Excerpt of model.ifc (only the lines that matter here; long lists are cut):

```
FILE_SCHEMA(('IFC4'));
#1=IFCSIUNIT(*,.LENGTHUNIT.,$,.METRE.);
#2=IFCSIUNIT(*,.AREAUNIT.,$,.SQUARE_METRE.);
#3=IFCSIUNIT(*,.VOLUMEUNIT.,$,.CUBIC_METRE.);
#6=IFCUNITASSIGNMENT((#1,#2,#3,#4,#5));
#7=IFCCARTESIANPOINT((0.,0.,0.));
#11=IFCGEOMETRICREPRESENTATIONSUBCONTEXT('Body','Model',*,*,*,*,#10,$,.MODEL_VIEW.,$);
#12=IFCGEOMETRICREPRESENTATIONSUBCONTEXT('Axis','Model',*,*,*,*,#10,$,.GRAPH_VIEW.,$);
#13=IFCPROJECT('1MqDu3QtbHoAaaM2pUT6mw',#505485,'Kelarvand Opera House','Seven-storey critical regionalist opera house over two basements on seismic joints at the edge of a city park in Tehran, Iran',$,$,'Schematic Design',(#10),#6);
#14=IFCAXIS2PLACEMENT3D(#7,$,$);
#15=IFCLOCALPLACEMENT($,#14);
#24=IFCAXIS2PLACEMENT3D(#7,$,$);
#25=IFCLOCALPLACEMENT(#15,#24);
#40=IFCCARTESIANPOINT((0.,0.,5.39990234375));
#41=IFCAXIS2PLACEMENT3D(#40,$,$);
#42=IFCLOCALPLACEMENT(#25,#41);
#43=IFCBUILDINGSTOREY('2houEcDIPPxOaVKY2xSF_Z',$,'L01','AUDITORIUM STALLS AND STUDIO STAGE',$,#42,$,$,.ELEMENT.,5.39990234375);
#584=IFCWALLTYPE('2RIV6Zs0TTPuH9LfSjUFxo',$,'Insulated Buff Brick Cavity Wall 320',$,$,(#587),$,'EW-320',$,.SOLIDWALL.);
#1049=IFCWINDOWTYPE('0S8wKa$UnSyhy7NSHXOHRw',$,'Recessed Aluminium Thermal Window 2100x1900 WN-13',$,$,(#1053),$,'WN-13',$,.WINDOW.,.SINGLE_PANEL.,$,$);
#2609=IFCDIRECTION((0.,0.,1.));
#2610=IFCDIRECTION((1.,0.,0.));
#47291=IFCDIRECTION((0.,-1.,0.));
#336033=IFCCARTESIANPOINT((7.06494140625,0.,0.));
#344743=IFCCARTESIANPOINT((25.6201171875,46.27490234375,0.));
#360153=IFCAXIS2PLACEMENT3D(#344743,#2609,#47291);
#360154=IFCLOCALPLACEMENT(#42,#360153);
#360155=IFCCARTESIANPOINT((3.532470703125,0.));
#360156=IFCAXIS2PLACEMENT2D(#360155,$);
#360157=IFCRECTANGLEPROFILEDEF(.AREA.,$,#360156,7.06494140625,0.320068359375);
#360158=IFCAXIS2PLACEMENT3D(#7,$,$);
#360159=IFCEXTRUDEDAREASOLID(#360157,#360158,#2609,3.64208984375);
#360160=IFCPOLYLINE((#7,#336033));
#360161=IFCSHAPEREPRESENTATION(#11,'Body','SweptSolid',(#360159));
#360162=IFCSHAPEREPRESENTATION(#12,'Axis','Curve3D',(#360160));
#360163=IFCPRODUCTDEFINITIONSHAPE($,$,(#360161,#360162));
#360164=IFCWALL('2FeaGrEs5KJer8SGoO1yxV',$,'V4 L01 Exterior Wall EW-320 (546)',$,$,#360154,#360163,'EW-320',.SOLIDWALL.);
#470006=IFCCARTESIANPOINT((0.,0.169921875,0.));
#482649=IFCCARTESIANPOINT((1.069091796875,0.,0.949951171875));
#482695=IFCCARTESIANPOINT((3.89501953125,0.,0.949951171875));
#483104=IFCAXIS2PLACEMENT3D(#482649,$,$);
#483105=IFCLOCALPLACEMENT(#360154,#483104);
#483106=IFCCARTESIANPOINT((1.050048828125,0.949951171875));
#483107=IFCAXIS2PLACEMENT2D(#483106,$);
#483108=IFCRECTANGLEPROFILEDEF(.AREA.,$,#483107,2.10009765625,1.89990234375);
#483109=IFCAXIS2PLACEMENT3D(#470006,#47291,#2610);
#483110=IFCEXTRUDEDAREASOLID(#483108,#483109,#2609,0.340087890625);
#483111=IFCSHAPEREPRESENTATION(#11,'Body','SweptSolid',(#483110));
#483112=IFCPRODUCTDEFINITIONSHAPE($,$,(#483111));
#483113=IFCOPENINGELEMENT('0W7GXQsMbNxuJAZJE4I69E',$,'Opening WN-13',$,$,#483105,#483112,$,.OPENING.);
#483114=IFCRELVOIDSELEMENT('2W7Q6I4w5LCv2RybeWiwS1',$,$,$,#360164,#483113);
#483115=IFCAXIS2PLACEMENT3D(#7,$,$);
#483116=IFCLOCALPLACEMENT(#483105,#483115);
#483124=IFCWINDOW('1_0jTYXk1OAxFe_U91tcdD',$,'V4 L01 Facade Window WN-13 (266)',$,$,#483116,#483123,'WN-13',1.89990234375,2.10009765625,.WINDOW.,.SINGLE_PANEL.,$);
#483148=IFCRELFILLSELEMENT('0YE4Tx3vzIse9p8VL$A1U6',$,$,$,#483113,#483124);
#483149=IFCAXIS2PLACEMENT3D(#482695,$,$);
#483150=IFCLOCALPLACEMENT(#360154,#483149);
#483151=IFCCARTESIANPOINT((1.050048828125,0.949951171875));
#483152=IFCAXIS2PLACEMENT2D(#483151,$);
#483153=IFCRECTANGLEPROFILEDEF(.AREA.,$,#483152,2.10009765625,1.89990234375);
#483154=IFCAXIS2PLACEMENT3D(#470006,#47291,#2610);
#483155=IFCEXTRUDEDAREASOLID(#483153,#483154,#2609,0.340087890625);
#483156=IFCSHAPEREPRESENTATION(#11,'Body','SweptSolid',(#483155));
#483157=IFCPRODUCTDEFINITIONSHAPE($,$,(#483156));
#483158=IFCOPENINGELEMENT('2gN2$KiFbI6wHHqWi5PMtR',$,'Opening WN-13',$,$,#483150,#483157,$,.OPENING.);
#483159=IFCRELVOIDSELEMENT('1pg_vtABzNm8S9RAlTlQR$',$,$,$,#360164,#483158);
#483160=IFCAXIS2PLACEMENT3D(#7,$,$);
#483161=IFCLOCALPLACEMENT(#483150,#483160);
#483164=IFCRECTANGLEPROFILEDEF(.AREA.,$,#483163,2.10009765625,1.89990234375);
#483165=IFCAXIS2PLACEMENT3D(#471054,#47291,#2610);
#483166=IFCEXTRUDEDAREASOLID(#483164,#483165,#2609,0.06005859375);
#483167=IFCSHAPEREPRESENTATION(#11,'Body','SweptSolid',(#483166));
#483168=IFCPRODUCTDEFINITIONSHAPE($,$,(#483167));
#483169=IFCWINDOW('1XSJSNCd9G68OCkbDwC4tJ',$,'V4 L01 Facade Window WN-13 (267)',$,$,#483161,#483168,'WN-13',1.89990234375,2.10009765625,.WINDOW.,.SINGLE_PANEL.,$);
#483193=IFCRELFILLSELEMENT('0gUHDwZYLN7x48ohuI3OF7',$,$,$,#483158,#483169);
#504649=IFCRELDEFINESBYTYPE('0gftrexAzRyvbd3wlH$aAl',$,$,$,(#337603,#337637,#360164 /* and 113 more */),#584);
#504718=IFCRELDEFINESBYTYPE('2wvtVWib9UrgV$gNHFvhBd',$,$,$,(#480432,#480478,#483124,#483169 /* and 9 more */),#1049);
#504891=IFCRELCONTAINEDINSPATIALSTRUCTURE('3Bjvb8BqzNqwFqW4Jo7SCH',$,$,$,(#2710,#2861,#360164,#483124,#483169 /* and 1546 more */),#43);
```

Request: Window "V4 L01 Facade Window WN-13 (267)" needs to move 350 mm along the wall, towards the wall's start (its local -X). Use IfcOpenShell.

```python
import ifcopenshell
import ifcopenshell.api.geometry
import ifcopenshell.util.placement

model = ifcopenshell.open("model.ifc")

window = model.by_guid("1XSJSNCd9G68OCkbDwC4tJ")
opening = window.FillsVoids[0].RelatingOpeningElement
wall = opening.VoidsElements[0].RelatingBuildingElement

wall_matrix = ifcopenshell.util.placement.get_local_placement(wall.ObjectPlacement)
shift = wall_matrix[:3, 0] * -0.35
before = ifcopenshell.util.placement.get_local_placement(window.ObjectPlacement)[:3, 3].copy()

# The window is placed relative to its opening, so it follows when the opening moves.
matrix = ifcopenshell.util.placement.get_local_placement(opening.ObjectPlacement)
matrix[:3, 3] += shift
ifcopenshell.api.geometry.edit_object_placement(
    model, product=opening, matrix=matrix, is_si=False, should_transform_children=True
)

after = ifcopenshell.util.placement.get_local_placement(window.ObjectPlacement)[:3, 3]
print("window moved by", (after - before).round(3) + 0.0)

model.write("model_rev.ifc")
```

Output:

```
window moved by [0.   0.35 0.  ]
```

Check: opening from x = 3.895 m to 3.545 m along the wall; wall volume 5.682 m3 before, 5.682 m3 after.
